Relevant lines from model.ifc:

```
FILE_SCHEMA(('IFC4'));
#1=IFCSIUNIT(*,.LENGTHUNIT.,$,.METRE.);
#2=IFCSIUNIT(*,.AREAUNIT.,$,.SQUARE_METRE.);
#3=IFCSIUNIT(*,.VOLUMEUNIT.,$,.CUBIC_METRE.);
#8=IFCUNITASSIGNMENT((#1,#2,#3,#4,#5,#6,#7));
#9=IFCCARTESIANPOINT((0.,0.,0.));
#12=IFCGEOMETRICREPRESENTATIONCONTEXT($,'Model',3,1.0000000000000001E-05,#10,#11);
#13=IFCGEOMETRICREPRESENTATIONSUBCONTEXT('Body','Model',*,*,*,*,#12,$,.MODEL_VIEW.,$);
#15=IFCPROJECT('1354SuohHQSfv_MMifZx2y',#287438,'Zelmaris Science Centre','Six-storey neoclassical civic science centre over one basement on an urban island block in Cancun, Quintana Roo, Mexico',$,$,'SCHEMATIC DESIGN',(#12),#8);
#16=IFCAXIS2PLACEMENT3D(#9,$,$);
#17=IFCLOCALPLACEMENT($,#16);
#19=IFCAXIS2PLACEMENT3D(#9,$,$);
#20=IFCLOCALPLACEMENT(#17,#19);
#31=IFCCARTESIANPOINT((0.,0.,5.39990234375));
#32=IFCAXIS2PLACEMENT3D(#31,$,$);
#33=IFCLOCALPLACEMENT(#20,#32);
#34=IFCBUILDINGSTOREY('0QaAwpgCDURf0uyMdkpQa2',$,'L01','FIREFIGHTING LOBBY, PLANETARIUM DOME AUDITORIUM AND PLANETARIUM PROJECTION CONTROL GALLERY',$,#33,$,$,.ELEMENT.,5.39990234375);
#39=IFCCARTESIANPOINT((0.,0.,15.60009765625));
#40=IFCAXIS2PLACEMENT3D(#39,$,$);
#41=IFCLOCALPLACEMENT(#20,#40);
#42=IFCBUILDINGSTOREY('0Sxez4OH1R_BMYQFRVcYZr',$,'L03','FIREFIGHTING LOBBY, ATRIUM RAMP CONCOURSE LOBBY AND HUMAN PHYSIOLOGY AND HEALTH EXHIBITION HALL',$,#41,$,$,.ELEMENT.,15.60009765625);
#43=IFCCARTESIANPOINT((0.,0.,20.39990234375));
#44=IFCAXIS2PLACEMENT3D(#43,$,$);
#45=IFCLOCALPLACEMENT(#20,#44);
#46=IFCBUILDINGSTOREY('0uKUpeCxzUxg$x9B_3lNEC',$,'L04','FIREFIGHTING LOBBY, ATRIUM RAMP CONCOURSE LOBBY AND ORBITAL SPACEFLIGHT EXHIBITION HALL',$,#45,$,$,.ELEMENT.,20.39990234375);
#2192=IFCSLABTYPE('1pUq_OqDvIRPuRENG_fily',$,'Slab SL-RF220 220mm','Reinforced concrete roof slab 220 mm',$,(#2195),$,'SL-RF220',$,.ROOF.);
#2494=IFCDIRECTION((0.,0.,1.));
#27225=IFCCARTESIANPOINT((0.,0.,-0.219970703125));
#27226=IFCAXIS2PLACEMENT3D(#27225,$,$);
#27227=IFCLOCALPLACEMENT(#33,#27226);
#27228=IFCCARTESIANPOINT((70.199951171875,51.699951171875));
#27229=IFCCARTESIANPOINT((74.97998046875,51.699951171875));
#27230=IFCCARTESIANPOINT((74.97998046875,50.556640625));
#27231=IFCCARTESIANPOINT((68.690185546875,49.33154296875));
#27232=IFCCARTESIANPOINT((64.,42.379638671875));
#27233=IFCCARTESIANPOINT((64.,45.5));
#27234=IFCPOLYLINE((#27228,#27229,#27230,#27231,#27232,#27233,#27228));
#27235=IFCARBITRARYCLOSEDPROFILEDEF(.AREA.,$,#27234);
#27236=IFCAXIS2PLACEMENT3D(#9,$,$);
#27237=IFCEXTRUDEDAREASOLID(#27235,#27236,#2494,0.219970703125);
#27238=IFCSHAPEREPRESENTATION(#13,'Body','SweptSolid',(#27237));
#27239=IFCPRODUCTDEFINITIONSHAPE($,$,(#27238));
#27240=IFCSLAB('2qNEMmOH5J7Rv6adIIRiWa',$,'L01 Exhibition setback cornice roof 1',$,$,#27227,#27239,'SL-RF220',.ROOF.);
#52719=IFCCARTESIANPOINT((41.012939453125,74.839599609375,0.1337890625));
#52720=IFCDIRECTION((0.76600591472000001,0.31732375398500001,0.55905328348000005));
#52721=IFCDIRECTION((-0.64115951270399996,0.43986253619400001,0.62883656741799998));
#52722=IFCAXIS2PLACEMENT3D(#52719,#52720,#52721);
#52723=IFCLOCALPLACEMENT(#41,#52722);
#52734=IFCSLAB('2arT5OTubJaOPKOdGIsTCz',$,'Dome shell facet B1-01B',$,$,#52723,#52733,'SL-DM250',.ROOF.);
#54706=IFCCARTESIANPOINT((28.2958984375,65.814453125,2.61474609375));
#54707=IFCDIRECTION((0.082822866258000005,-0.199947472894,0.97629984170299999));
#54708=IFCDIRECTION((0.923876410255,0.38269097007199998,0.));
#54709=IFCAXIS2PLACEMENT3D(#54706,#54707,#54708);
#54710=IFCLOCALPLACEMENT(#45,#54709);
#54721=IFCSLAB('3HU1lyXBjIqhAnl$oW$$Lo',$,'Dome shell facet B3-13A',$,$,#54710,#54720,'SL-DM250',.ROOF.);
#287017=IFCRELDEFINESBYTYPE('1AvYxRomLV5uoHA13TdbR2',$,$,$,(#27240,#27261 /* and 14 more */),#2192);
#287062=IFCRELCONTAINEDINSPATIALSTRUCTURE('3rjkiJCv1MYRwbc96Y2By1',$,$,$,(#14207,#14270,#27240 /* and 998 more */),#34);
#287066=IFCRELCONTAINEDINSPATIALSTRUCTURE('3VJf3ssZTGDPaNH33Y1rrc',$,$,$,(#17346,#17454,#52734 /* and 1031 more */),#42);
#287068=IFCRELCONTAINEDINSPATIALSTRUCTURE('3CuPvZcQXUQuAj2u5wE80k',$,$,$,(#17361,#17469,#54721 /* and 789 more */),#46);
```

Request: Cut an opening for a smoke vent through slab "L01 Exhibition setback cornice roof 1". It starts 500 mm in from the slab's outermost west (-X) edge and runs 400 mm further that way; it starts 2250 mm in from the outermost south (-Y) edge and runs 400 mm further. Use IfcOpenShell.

```python
import numpy as np
import ifcopenshell
import ifcopenshell.api.feature
import ifcopenshell.api.geometry
import ifcopenshell.api.root
import ifcopenshell.geom
import ifcopenshell.util.placement
import ifcopenshell.util.representation
import ifcopenshell.util.shape
import ifcopenshell.util.unit

model = ifcopenshell.open("model.ifc")
unit_scale = ifcopenshell.util.unit.calculate_unit_scale(model)
settings = ifcopenshell.geom.settings()


def volume(element):
    """Net volume in cubic metres, openings subtracted."""
    shape = ifcopenshell.geom.create_shape(settings, element)
    return ifcopenshell.util.shape.get_volume(shape.geometry)


slab = model.by_guid("2qNEMmOH5J7Rv6adIIRiWa")
before = volume(slab)

# Extent in the slab's own axes, in metres. The edges named are its -X and -Y sides.
slab_shape = ifcopenshell.geom.create_shape(settings, slab)
vertices = ifcopenshell.util.shape.get_vertices(slab_shape.geometry)
x_min, y_min, bottom = vertices.min(axis=0)
top = vertices[:, 2].max()

opening = ifcopenshell.api.root.create_entity(model, ifc_class="IfcOpeningElement", name="Smoke vent opening", predefined_type="OPENING")
context = ifcopenshell.util.representation.get_context(model, "Model", "Body", "MODEL_VIEW")
width, depth = 0.4, 0.4
outline = [(0.0, 0.0), (width, 0.0), (width, depth), (0.0, depth), (0.0, 0.0)]
# Overshoot both faces by 50 mm so the cut is clean.
shape = ifcopenshell.api.geometry.add_slab_representation(
    model, context=context, depth=top - bottom + 0.1, polyline=outline
)
ifcopenshell.api.geometry.assign_representation(model, product=opening, representation=shape)

matrix = ifcopenshell.util.placement.get_local_placement(slab.ObjectPlacement)
matrix[:, 3] = matrix @ np.append(np.array([x_min + 0.5, y_min + 2.25, bottom - 0.05]) / unit_scale, 1.0)
ifcopenshell.api.geometry.edit_object_placement(model, product=opening, matrix=matrix, is_si=False)
ifcopenshell.api.feature.add_feature(model, feature=opening, element=slab)

after = volume(slab)

print(f"slab volume {before:.3f} -> {after:.3f} m3")

model.write("model-out.ifc")
```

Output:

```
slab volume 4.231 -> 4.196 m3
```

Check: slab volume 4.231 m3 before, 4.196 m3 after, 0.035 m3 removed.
